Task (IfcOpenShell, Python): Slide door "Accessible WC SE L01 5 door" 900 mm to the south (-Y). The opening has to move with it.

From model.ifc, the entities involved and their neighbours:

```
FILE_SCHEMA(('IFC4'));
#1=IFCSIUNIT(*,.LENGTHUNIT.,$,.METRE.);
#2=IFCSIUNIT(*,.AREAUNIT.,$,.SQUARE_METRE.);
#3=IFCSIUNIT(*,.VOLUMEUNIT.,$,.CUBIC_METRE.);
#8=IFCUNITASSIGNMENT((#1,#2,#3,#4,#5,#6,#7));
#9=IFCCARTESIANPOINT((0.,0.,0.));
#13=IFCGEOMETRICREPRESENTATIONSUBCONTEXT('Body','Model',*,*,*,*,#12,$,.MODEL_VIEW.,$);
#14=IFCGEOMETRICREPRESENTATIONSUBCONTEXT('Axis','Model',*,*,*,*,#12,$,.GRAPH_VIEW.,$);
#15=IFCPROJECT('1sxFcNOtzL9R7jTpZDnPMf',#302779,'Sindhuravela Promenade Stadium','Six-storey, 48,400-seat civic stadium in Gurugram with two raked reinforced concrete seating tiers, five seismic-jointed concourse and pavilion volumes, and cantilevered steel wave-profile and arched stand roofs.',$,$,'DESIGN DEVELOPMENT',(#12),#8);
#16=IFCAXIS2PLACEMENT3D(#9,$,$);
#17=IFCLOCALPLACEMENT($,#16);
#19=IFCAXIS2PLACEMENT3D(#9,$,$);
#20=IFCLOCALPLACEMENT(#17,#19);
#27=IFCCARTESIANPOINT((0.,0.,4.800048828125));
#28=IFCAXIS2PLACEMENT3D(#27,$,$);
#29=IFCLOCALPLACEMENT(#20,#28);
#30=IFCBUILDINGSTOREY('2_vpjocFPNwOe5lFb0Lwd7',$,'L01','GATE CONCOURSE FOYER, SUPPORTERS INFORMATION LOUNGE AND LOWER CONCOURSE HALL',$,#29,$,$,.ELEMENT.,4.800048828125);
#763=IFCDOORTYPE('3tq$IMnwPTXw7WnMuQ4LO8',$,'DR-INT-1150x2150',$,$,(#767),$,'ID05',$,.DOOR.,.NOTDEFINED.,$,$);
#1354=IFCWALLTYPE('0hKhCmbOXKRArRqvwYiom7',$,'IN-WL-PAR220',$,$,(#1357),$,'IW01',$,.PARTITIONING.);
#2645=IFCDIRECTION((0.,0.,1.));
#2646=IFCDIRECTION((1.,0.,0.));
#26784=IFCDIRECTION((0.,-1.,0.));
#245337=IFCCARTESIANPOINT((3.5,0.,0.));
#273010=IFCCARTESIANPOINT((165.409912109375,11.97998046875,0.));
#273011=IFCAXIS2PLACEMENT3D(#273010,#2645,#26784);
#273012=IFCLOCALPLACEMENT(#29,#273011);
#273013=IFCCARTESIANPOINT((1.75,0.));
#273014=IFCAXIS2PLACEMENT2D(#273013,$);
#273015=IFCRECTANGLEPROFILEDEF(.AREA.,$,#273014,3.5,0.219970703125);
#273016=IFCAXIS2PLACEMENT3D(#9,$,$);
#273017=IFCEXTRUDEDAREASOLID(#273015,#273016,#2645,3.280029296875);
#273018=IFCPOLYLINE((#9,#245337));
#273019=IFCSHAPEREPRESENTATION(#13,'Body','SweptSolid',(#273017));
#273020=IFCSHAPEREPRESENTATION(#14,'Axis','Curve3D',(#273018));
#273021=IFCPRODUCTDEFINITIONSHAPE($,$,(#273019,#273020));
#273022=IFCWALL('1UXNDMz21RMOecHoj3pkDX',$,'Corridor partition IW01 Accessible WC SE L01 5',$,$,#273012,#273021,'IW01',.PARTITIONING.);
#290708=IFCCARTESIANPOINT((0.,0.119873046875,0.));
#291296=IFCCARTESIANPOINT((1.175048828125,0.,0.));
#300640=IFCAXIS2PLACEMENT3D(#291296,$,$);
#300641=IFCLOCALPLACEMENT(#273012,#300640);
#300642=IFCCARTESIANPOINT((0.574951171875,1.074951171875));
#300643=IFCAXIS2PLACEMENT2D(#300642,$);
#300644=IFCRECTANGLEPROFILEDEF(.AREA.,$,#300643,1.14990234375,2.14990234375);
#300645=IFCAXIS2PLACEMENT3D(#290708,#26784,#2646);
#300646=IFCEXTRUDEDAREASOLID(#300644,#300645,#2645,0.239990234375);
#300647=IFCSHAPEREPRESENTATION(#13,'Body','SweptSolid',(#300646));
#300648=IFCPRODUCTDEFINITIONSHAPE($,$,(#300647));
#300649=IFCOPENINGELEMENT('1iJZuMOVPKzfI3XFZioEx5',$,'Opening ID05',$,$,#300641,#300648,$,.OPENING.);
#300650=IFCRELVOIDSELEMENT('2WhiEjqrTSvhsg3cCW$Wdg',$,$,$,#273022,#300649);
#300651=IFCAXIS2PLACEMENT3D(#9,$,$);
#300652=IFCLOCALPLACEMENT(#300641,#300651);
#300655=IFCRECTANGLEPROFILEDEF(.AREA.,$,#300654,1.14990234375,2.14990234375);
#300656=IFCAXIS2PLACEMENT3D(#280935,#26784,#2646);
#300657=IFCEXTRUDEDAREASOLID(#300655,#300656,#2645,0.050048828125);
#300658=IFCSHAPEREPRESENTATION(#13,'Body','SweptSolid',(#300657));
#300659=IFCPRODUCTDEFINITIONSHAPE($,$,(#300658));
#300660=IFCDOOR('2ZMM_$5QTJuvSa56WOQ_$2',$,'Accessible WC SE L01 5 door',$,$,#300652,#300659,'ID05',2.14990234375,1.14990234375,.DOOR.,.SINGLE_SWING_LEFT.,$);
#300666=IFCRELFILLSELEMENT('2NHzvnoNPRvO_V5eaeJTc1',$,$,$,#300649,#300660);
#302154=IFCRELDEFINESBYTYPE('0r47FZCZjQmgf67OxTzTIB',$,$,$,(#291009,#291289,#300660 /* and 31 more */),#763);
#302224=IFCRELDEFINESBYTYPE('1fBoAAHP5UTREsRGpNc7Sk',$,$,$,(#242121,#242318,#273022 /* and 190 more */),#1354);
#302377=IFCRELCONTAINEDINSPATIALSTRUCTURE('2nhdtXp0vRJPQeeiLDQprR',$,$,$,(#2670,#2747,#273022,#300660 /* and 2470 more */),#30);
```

```python
import ifcopenshell
import ifcopenshell.api.geometry
import ifcopenshell.util.placement
import ifcopenshell.util.unit

model = ifcopenshell.open("model.ifc")
unit_scale = ifcopenshell.util.unit.calculate_unit_scale(model)

door = model.by_guid("2ZMM_$5QTJuvSa56WOQ_$2")
opening = door.FillsVoids[0].RelatingOpeningElement
wall = opening.VoidsElements[0].RelatingBuildingElement

wall_matrix = ifcopenshell.util.placement.get_local_placement(wall.ObjectPlacement)
shift = wall_matrix[:3, 0] * 0.9 / unit_scale
before = ifcopenshell.util.placement.get_local_placement(door.ObjectPlacement)[:3, 3].copy()

# The door is placed relative to its opening, so it follows when the opening moves.
matrix = ifcopenshell.util.placement.get_local_placement(opening.ObjectPlacement)
matrix[:3, 3] += shift
ifcopenshell.api.geometry.edit_object_placement(
    model, product=opening, matrix=matrix, is_si=False, should_transform_children=True
)

after = ifcopenshell.util.placement.get_local_placement(door.ObjectPlacement)[:3, 3]
print("door moved by", (after - before).round(3) + 0.0)

model.write("model_edited.ifc")
```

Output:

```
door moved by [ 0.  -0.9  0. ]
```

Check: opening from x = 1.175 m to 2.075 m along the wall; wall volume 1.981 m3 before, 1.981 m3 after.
